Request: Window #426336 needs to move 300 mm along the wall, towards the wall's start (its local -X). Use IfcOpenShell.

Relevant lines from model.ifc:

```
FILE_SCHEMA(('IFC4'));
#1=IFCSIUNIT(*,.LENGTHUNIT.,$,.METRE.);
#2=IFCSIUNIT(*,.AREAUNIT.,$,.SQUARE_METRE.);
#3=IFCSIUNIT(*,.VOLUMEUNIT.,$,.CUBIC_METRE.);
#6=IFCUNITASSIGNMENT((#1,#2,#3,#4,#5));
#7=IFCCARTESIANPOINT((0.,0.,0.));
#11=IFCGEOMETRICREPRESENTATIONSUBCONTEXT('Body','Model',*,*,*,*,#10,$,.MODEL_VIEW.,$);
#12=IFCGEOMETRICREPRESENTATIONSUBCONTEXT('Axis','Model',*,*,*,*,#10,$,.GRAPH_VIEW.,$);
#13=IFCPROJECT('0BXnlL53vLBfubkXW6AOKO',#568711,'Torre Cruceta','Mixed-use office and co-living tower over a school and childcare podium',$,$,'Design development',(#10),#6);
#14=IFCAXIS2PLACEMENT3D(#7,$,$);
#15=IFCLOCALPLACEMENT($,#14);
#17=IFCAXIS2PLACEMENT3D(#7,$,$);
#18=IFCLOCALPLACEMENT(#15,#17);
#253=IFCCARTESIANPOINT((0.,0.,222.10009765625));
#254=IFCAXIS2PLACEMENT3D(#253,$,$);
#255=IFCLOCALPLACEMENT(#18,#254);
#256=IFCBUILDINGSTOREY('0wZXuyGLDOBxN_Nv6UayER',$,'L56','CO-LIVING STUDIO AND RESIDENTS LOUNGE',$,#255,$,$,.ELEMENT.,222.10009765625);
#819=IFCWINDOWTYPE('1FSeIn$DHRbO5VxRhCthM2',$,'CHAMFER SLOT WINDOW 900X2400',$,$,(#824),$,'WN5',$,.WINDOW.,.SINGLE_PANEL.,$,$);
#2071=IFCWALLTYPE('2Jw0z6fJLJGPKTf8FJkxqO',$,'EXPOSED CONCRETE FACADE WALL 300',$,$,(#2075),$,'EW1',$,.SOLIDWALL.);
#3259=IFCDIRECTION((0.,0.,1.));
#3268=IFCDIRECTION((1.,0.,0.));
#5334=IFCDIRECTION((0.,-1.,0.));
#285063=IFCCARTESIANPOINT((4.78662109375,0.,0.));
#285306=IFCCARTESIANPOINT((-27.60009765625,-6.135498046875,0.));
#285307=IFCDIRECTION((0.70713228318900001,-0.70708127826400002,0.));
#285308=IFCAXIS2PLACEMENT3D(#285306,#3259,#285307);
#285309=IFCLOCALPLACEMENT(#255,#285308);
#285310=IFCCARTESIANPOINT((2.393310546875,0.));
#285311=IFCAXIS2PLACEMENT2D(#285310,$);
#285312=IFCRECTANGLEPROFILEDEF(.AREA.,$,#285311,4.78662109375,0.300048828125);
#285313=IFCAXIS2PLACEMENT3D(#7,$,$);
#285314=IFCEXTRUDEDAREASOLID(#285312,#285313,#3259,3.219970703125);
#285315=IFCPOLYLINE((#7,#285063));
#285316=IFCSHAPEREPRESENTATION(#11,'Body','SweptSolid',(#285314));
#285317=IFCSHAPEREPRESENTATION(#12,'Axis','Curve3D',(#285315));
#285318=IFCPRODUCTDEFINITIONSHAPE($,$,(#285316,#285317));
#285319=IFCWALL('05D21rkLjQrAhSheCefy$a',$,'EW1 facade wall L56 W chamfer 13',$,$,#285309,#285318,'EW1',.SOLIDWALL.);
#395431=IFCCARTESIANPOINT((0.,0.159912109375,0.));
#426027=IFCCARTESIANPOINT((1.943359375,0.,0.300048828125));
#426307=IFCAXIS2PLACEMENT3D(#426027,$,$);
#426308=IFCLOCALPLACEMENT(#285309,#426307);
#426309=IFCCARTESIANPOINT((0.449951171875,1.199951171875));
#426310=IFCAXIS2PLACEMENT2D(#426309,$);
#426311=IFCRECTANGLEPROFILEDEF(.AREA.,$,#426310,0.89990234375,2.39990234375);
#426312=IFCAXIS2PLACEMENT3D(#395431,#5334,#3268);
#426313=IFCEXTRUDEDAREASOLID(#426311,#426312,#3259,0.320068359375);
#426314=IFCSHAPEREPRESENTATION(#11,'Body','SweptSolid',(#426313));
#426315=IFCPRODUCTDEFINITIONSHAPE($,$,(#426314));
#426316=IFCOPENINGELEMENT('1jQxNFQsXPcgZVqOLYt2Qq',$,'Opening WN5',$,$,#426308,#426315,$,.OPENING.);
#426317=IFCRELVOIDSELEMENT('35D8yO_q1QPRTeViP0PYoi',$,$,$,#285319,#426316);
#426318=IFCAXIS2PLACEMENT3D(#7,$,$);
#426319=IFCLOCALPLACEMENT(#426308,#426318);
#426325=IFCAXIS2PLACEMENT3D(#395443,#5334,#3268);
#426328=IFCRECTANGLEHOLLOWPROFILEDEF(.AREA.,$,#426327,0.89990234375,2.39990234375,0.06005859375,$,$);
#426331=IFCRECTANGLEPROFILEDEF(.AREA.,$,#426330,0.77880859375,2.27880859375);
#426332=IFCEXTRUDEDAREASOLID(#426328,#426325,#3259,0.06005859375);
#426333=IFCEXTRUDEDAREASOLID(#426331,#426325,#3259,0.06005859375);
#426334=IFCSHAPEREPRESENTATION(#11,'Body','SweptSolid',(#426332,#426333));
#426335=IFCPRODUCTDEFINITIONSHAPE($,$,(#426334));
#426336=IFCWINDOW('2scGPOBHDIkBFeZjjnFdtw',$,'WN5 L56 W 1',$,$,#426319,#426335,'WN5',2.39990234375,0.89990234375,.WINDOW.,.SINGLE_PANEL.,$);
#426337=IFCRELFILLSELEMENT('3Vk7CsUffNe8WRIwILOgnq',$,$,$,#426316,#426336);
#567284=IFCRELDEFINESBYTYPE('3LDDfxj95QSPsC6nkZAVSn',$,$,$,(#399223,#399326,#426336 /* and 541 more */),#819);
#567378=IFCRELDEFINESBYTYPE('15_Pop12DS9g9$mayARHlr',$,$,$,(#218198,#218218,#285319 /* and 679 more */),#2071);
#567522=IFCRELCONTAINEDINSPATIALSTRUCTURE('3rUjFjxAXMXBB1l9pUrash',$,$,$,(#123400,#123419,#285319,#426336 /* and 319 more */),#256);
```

```python
import ifcopenshell
import ifcopenshell.api.geometry
import ifcopenshell.util.placement
import ifcopenshell.util.unit

model = ifcopenshell.open("model.ifc")
unit_scale = ifcopenshell.util.unit.calculate_unit_scale(model)

window = model.by_guid("2scGPOBHDIkBFeZjjnFdtw")
opening = window.FillsVoids[0].RelatingOpeningElement
wall = opening.VoidsElements[0].RelatingBuildingElement

wall_matrix = ifcopenshell.util.placement.get_local_placement(wall.ObjectPlacement)
shift = wall_matrix[:3, 0] * -0.3 / unit_scale
before = ifcopenshell.util.placement.get_local_placement(window.ObjectPlacement)[:3, 3].copy()

# The window is placed relative to its opening, so it follows when the opening moves.
matrix = ifcopenshell.util.placement.get_local_placement(opening.ObjectPlacement)
matrix[:3, 3] += shift
ifcopenshell.api.geometry.edit_object_placement(
    model, product=opening, matrix=matrix, is_si=False, should_transform_children=True
)

after = ifcopenshell.util.placement.get_local_placement(window.ObjectPlacement)[:3, 3]
print("window moved by", (after - before).round(3) + 0.0)

model.write("model-out.ifc")
```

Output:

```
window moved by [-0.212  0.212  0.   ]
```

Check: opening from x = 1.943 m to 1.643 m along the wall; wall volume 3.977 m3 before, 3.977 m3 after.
